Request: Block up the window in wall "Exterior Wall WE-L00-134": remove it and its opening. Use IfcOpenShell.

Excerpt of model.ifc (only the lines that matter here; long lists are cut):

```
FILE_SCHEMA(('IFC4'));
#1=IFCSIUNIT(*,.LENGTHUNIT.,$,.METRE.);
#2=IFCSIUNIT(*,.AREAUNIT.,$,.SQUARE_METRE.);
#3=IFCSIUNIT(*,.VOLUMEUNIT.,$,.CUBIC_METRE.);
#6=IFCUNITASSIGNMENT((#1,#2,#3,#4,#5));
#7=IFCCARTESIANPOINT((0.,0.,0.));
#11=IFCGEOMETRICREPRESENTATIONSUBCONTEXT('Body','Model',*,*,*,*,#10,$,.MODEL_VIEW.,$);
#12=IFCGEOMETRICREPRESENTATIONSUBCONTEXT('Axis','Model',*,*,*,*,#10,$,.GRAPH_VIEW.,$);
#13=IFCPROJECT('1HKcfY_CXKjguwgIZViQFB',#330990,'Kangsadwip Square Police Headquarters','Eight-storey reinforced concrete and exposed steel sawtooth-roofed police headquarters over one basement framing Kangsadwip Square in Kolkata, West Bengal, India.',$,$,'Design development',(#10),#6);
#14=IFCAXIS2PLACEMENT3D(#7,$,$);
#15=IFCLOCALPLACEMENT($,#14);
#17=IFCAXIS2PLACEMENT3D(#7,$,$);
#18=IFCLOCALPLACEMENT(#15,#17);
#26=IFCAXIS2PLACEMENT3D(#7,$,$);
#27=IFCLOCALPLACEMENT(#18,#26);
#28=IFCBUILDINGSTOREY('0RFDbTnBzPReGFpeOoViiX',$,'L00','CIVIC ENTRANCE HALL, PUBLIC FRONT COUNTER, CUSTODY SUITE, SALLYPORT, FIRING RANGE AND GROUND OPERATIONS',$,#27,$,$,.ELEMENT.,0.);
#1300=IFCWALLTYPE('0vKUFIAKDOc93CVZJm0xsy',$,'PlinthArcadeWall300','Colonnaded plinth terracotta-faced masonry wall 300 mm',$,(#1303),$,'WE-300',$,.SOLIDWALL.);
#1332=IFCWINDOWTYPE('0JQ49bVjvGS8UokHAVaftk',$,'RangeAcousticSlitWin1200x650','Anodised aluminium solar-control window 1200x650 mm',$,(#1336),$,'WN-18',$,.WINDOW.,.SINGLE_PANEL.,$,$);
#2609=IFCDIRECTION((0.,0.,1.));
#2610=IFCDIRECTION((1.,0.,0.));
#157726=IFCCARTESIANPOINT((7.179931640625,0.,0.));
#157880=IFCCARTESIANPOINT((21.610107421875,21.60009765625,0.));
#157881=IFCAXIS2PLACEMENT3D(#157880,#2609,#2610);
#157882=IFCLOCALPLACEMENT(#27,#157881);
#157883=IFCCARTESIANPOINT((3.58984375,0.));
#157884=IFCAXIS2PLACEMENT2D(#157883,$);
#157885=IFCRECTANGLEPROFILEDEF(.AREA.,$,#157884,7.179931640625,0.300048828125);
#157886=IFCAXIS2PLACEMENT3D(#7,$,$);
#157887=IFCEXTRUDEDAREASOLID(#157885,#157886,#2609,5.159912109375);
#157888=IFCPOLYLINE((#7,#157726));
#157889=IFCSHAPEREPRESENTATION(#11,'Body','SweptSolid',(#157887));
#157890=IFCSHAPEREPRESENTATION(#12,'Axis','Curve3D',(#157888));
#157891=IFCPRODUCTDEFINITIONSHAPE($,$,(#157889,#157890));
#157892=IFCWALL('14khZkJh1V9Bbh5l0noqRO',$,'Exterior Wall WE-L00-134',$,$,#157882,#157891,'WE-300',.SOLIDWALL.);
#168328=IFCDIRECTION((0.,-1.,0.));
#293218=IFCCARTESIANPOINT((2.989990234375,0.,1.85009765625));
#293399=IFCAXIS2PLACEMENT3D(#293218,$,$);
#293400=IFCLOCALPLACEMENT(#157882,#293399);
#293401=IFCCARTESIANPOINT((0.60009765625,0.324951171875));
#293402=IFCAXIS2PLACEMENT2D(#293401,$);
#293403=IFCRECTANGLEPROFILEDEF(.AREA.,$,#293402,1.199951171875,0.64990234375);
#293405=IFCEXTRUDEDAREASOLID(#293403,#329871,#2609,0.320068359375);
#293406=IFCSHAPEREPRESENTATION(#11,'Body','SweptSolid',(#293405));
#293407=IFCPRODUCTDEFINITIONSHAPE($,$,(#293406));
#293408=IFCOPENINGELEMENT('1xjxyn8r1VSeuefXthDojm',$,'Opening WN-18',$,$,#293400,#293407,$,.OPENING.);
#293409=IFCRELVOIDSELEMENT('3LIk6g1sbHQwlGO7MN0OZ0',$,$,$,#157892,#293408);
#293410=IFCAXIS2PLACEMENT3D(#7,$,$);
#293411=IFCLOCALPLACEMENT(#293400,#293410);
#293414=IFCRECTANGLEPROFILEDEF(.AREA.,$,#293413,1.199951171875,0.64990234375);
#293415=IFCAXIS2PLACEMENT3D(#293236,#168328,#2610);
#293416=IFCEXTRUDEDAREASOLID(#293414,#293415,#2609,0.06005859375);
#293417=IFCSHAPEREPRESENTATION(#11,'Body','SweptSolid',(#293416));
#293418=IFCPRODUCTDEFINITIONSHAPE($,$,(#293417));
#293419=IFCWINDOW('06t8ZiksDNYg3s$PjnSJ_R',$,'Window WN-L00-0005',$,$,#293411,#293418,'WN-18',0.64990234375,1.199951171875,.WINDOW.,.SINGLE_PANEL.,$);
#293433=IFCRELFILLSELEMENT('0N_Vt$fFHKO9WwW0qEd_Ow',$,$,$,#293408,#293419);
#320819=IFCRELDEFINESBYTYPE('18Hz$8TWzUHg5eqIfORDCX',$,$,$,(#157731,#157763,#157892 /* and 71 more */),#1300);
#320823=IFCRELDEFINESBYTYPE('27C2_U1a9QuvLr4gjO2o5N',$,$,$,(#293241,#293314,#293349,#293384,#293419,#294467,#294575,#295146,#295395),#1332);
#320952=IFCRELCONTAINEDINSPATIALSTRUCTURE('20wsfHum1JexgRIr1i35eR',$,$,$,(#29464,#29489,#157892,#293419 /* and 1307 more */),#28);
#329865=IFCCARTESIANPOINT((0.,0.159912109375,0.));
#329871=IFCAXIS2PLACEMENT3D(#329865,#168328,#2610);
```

```python
import ifcopenshell
import ifcopenshell.api.feature
import ifcopenshell.api.root
import ifcopenshell.geom
import ifcopenshell.util.shape

model = ifcopenshell.open("model.ifc")
settings = ifcopenshell.geom.settings()


def volume(element):
    """Net volume in cubic metres, openings subtracted."""
    shape = ifcopenshell.geom.create_shape(settings, element)
    return ifcopenshell.util.shape.get_volume(shape.geometry)


window = model.by_guid("06t8ZiksDNYg3s$PjnSJ_R")
opening = window.FillsVoids[0].RelatingOpeningElement
wall = opening.VoidsElements[0].RelatingBuildingElement
before = volume(wall)

ifcopenshell.api.root.remove_product(model, product=window)
ifcopenshell.api.feature.remove_feature(model, feature=opening)

after = volume(wall)

print(f"wall volume {before:.3f} -> {after:.3f} m3")

model.write("model_updated.ifc")
```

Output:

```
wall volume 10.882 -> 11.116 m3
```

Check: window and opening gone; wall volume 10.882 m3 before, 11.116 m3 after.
